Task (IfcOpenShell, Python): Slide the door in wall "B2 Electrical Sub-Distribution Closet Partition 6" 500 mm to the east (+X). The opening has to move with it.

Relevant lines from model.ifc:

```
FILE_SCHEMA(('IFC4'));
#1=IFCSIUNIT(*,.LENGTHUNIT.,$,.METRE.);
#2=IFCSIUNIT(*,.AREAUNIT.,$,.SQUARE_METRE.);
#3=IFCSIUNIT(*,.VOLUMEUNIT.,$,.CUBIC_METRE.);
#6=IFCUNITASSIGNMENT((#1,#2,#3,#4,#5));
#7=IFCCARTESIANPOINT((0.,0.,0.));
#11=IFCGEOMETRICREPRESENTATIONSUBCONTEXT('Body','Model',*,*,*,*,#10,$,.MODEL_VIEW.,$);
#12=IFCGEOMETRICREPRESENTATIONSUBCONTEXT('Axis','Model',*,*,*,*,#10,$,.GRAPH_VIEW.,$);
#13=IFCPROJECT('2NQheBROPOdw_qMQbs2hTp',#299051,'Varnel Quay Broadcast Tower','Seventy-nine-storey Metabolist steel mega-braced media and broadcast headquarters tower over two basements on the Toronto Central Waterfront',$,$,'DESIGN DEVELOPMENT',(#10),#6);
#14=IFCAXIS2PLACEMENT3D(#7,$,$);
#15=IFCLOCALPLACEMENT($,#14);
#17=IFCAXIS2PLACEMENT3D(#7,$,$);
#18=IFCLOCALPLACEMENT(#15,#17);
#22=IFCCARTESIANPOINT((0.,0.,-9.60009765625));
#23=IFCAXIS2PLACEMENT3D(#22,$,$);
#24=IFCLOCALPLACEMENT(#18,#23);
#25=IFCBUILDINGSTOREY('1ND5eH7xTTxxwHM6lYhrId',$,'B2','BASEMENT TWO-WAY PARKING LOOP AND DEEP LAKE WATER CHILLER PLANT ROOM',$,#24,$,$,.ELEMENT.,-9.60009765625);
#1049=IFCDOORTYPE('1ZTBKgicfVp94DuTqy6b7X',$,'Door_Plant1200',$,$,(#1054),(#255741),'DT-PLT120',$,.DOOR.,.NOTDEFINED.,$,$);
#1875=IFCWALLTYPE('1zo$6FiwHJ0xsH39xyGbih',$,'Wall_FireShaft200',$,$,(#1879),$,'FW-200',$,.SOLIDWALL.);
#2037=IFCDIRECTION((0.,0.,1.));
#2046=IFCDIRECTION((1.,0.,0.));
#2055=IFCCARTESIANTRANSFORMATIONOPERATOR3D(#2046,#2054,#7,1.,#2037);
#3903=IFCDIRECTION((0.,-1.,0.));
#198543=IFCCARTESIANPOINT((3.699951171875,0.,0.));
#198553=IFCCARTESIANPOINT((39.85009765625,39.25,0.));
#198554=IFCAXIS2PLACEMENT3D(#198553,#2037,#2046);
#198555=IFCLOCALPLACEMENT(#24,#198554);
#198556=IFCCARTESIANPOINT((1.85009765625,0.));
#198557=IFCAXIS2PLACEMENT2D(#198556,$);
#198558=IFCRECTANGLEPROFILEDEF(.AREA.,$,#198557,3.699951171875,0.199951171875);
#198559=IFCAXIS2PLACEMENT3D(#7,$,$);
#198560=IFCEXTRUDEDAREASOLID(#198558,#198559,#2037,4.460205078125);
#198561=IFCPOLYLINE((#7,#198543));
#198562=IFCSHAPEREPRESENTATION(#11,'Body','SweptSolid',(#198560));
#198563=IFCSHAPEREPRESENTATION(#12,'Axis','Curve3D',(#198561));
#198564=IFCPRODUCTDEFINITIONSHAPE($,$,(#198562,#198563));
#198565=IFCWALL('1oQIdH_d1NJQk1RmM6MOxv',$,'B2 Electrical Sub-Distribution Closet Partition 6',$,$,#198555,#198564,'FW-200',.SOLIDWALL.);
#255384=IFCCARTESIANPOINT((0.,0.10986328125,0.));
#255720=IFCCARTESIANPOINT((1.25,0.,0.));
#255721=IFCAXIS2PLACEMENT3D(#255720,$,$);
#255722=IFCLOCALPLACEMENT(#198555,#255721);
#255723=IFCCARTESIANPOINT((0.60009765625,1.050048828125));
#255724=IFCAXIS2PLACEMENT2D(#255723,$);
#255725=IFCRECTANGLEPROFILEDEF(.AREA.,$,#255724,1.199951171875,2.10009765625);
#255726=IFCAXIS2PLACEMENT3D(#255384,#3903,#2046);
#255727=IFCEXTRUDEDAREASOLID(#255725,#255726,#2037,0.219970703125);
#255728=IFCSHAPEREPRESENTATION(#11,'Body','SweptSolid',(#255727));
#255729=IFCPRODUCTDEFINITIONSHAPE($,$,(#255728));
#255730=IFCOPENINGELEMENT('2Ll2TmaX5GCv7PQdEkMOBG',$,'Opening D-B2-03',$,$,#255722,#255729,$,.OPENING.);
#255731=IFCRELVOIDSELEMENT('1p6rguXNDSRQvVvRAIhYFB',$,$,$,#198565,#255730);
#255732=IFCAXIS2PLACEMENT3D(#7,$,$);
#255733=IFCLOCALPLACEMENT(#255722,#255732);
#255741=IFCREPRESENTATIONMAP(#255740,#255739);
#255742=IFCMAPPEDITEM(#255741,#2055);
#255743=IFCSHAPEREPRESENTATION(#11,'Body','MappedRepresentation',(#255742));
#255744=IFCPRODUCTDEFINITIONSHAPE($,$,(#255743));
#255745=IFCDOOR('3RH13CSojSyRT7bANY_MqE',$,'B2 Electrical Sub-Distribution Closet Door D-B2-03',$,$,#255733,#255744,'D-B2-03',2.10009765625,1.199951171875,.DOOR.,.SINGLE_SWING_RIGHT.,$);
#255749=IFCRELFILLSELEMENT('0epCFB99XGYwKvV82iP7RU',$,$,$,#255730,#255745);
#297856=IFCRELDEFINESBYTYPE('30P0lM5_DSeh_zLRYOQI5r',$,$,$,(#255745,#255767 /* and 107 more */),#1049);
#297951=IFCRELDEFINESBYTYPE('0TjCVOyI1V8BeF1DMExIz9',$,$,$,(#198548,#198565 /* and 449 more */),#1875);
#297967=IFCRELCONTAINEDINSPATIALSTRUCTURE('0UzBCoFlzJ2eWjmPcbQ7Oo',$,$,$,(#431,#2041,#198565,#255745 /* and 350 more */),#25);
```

```python
import ifcopenshell
import ifcopenshell.api.geometry
import ifcopenshell.util.placement
import ifcopenshell.util.unit

model = ifcopenshell.open("model.ifc")
unit_scale = ifcopenshell.util.unit.calculate_unit_scale(model)

door = model.by_guid("3RH13CSojSyRT7bANY_MqE")
opening = door.FillsVoids[0].RelatingOpeningElement
wall = opening.VoidsElements[0].RelatingBuildingElement

wall_matrix = ifcopenshell.util.placement.get_local_placement(wall.ObjectPlacement)
shift = wall_matrix[:3, 0] * 0.5 / unit_scale
before = ifcopenshell.util.placement.get_local_placement(door.ObjectPlacement)[:3, 3].copy()

# The door is placed relative to its opening, so it follows when the opening moves.
matrix = ifcopenshell.util.placement.get_local_placement(opening.ObjectPlacement)
matrix[:3, 3] += shift
ifcopenshell.api.geometry.edit_object_placement(
    model, product=opening, matrix=matrix, is_si=False, should_transform_children=True
)

after = ifcopenshell.util.placement.get_local_placement(door.ObjectPlacement)[:3, 3]
print("door moved by", (after - before).round(3) + 0.0)

model.write("model_edited.ifc")
```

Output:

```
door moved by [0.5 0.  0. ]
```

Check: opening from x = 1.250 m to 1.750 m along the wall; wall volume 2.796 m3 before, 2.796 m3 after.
